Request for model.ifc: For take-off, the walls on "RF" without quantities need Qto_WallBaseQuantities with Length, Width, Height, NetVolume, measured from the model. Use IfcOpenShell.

First a look at what the model holds.

```python
import ifcopenshell
import ifcopenshell.util.element
import ifcopenshell.util.unit

model = ifcopenshell.open("model.ifc")
print(model.schema)
for unit_type in ("LENGTHUNIT", "AREAUNIT", "VOLUMEUNIT"):
    print(unit_type, ifcopenshell.util.unit.calculate_unit_scale(model, unit_type))
storey = next(s for s in model.by_type("IfcBuildingStorey") if s.Name == "RF")
walls = [e for e in ifcopenshell.util.element.get_decomposition(storey) if e.is_a("IfcWall")]
for e in sorted(walls, key=lambda e: e.id()):
    print(e.id(), e.is_a(), e.Name, list(ifcopenshell.util.element.get_psets(e, qtos_only=True)), sep=" | ")
```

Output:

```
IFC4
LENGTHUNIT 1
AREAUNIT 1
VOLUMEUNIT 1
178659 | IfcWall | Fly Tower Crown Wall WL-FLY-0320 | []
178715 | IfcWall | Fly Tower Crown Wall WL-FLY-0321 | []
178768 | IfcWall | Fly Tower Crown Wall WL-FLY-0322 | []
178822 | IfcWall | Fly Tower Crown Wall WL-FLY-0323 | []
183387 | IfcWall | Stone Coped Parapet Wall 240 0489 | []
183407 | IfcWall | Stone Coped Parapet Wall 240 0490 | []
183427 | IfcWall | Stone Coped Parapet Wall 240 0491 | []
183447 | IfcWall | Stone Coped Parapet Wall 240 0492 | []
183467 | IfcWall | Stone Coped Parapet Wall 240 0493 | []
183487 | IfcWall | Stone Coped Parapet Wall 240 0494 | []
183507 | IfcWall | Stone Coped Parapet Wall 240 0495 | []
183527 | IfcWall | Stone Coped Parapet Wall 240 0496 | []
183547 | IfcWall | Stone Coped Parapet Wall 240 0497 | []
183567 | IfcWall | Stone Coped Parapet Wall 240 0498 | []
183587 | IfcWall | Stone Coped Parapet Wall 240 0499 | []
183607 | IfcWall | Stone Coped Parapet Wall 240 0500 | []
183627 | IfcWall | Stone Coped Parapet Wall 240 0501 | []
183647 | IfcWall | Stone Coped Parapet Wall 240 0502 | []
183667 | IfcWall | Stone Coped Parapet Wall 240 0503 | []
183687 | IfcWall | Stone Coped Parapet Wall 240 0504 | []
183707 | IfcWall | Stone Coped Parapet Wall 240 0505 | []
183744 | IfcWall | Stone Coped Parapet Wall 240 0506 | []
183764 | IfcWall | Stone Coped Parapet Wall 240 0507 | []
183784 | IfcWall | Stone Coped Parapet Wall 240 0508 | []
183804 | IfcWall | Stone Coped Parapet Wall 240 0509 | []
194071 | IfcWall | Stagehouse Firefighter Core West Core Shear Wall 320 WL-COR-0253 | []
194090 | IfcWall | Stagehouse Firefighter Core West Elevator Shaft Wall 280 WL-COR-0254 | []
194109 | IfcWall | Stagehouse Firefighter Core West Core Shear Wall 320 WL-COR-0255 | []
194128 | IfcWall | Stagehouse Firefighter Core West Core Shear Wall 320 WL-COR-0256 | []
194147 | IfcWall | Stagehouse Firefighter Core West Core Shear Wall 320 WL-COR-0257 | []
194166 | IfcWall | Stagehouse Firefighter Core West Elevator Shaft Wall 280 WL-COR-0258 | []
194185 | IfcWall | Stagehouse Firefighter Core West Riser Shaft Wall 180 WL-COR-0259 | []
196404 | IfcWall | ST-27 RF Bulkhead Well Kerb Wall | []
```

```python
import ifcopenshell
import ifcopenshell.api.pset
import ifcopenshell.geom
import ifcopenshell.util.element
import ifcopenshell.util.shape
import ifcopenshell.util.unit

model = ifcopenshell.open("model.ifc")
unit_scale = ifcopenshell.util.unit.calculate_unit_scale(model)
volume_scale = ifcopenshell.util.unit.calculate_unit_scale(model, "VOLUMEUNIT")
settings = ifcopenshell.geom.settings()

storey = next(s for s in model.by_type("IfcBuildingStorey") if s.Name == "RF")
walls = [e for e in ifcopenshell.util.element.get_decomposition(storey) if e.is_a("IfcWall")]

for e in sorted(walls, key=lambda e: e.id()):
    if ifcopenshell.util.element.get_psets(e, qtos_only=True, should_inherit=False):
        continue
    # Geometry comes back in metres, in the element's own axes.
    shape = ifcopenshell.geom.create_shape(settings, e)
    values = {
        "Length": ifcopenshell.util.shape.get_x(shape.geometry) / unit_scale,
        "Width": ifcopenshell.util.shape.get_y(shape.geometry) / unit_scale,
        "Height": ifcopenshell.util.shape.get_z(shape.geometry) / unit_scale,
        "NetVolume": ifcopenshell.util.shape.get_volume(shape.geometry) / volume_scale,
    }
    qto = ifcopenshell.api.pset.add_qto(model, product=e, name="Qto_WallBaseQuantities")
    ifcopenshell.api.pset.edit_qto(model, qto=qto, properties=values)
    print(e.id(), {k: round(v, 3) for k, v in values.items()})

model.write("model_rev.ifc")
```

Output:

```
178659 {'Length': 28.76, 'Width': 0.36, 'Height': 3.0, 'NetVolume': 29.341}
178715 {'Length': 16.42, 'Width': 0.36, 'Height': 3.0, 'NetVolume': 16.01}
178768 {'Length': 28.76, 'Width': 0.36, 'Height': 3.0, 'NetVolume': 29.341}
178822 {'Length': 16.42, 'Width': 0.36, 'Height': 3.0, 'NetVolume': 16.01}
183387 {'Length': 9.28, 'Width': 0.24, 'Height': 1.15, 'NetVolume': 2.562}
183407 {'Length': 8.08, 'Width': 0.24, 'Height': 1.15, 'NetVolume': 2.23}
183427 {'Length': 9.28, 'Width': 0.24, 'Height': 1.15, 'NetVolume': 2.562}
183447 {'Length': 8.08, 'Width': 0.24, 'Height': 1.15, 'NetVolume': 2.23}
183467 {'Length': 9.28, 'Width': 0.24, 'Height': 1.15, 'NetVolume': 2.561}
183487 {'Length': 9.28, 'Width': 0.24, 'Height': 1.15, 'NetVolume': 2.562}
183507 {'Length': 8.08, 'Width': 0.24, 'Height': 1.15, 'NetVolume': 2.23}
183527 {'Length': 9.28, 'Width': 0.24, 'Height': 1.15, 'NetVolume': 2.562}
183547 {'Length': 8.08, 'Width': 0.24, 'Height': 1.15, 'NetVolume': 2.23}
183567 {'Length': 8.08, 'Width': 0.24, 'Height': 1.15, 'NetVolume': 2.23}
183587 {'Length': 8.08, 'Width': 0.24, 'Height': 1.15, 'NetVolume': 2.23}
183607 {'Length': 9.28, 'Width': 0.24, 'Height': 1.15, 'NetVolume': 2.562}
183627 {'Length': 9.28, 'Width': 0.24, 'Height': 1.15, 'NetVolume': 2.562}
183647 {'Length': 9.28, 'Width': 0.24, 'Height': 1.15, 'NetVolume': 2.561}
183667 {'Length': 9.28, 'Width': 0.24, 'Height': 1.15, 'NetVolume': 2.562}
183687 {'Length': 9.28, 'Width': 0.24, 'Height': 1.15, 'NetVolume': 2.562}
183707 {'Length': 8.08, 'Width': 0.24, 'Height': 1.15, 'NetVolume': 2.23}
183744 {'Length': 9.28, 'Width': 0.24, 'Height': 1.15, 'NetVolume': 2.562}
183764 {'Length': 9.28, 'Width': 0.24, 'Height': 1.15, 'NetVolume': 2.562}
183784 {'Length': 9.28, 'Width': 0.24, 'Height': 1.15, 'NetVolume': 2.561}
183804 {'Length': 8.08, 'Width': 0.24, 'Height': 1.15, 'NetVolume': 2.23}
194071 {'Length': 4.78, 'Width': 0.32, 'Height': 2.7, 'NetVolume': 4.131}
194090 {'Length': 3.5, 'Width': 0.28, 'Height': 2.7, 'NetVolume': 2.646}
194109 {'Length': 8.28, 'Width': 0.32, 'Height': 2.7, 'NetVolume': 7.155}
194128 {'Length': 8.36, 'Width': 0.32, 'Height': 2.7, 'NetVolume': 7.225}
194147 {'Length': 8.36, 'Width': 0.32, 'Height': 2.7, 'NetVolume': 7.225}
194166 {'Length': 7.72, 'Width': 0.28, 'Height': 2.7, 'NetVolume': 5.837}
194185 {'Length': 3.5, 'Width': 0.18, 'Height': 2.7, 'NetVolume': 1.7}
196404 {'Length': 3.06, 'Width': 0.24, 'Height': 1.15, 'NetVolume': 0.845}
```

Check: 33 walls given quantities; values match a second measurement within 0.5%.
